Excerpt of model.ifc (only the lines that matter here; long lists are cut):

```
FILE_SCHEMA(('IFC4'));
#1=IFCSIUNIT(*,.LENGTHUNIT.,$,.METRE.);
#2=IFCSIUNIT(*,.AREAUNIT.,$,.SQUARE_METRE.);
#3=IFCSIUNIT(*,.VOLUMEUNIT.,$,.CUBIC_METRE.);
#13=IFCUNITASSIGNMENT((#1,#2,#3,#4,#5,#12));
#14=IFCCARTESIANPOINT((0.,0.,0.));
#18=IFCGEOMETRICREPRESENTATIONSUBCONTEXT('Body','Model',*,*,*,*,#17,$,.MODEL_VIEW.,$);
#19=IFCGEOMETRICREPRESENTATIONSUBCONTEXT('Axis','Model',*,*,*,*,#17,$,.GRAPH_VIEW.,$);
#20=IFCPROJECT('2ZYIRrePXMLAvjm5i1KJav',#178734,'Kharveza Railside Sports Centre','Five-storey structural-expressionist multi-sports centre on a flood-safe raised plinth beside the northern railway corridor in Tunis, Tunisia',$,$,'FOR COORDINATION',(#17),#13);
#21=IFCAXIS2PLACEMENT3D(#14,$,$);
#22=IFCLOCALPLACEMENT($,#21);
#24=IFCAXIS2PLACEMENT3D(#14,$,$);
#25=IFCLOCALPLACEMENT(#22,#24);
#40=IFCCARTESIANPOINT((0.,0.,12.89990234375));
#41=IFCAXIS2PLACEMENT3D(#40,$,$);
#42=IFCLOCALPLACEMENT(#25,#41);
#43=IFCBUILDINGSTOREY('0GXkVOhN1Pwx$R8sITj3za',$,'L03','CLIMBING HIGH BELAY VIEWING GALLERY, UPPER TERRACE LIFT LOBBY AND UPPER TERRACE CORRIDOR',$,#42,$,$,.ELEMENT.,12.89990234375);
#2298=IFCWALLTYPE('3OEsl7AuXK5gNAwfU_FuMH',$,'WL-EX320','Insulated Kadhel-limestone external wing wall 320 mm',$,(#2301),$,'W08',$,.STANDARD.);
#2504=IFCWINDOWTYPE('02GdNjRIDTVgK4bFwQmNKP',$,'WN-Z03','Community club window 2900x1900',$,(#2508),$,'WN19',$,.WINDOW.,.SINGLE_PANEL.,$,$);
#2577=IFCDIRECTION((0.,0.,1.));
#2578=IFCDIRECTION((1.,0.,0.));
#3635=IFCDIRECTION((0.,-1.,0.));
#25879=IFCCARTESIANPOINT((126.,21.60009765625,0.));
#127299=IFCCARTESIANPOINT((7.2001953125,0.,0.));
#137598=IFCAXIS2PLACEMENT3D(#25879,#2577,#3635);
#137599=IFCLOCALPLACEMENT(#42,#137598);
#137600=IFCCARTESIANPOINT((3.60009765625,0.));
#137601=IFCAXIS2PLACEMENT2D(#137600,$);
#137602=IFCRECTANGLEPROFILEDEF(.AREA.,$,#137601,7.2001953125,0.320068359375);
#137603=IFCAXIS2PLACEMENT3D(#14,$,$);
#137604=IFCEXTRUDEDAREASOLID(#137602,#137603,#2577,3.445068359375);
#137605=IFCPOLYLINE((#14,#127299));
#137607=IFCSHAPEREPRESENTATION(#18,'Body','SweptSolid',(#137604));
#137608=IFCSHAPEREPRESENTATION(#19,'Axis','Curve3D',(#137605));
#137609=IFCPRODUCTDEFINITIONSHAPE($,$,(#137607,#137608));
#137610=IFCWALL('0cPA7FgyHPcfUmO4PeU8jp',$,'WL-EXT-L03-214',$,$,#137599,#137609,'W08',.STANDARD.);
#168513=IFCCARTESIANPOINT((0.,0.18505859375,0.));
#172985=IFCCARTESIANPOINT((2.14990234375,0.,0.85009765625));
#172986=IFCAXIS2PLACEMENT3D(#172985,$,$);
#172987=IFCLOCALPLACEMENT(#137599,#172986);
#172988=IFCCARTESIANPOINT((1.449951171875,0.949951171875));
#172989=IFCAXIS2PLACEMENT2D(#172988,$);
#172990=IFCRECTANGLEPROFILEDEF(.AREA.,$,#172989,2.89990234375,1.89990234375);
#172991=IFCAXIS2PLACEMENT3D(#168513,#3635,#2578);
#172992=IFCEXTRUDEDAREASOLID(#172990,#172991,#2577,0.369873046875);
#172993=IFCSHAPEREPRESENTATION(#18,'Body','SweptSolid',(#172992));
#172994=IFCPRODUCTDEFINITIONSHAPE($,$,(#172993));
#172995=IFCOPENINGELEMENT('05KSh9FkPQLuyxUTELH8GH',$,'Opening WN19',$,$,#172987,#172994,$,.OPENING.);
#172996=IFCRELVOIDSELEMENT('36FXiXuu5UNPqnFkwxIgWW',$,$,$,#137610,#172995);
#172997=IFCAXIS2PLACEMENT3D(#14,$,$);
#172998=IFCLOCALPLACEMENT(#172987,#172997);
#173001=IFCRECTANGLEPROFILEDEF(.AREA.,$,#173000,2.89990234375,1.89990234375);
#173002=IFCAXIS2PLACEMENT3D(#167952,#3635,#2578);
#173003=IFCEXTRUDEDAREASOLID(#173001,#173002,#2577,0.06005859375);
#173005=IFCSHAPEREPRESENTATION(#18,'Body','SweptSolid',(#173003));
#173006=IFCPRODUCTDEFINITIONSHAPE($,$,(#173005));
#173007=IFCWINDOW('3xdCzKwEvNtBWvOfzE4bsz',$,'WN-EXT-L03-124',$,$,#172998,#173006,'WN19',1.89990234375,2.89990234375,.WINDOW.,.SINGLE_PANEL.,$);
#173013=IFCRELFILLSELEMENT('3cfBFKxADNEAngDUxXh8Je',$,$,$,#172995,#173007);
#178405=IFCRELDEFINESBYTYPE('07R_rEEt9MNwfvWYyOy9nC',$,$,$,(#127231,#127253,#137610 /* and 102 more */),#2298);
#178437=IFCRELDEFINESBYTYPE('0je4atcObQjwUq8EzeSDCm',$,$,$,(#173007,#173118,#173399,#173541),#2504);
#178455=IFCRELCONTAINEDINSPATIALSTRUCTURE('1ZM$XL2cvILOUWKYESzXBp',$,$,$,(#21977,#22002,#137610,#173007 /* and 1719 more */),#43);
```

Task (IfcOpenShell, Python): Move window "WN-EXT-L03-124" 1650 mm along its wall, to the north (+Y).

```python
import ifcopenshell
import ifcopenshell.api.geometry
import ifcopenshell.util.placement
import ifcopenshell.util.unit

model = ifcopenshell.open("model.ifc")
unit_scale = ifcopenshell.util.unit.calculate_unit_scale(model)

window = model.by_guid("3xdCzKwEvNtBWvOfzE4bsz")
opening = window.FillsVoids[0].RelatingOpeningElement
wall = opening.VoidsElements[0].RelatingBuildingElement

wall_matrix = ifcopenshell.util.placement.get_local_placement(wall.ObjectPlacement)
shift = wall_matrix[:3, 0] * -1.65 / unit_scale
before = ifcopenshell.util.placement.get_local_placement(window.ObjectPlacement)[:3, 3].copy()

# The window is placed relative to its opening, so it follows when the opening moves.
matrix = ifcopenshell.util.placement.get_local_placement(opening.ObjectPlacement)
matrix[:3, 3] += shift
ifcopenshell.api.geometry.edit_object_placement(
    model, product=opening, matrix=matrix, is_si=False, should_transform_children=True
)

after = ifcopenshell.util.placement.get_local_placement(window.ObjectPlacement)[:3, 3]
print("window moved by", (after - before).round(3) + 0.0)

model.write("model_updated.ifc")
```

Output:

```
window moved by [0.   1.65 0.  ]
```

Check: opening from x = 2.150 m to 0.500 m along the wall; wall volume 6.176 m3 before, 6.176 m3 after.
